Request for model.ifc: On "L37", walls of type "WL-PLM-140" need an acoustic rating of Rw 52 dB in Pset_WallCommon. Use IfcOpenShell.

First a look at what the model holds.

```python
import ifcopenshell
import ifcopenshell.util.element

model = ifcopenshell.open("model.ifc")
print(model.schema)
storey = next(s for s in model.by_type("IfcBuildingStorey") if s.Name == "L37")
walls = [e for e in ifcopenshell.util.element.get_decomposition(storey) if e.is_a("IfcWall")]
seen = {}
for e in walls:
    element_type = ifcopenshell.util.element.get_type(e)
    key = (element_type.Name if element_type != e and element_type else None, ifcopenshell.util.element.get_pset(e, "Pset_WallCommon", "AcousticRating"))
    seen[key] = seen.get(key, 0) + 1
for (name, value), count in sorted(seen.items(), key=str):
    print(count, "x", name, "|", value)
```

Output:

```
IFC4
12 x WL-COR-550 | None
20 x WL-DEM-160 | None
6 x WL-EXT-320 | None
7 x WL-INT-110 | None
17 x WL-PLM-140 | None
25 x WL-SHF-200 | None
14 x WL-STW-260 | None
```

```python
import ifcopenshell
import ifcopenshell.api.pset
import ifcopenshell.util.element

model = ifcopenshell.open("model.ifc")

storey = next(s for s in model.by_type("IfcBuildingStorey") if s.Name == "L37")
walls = [e for e in ifcopenshell.util.element.get_decomposition(storey) if e.is_a("IfcWall")]

count = 0
for e in walls:
    element_type = ifcopenshell.util.element.get_type(e)
    if element_type in (None, e) or element_type.Name != "WL-PLM-140":
        continue
    found = ifcopenshell.util.element.get_pset(e, "Pset_WallCommon", should_inherit=False)
    if found:
        pset = model.by_id(found["id"])
        if len(ifcopenshell.util.element.get_elements_by_pset(pset)) > 1:
            pset = ifcopenshell.api.pset.unshare_pset(model, products=[e], pset=pset)[0]
    else:
        pset = ifcopenshell.api.pset.add_pset(model, product=e, name="Pset_WallCommon")
    ifcopenshell.api.pset.edit_pset(model, pset=pset, properties={"AcousticRating": "Rw 52 dB"})
    count += 1

print(count, "walls updated")

model.write("model_v2.ifc")
```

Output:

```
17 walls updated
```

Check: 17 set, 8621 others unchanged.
